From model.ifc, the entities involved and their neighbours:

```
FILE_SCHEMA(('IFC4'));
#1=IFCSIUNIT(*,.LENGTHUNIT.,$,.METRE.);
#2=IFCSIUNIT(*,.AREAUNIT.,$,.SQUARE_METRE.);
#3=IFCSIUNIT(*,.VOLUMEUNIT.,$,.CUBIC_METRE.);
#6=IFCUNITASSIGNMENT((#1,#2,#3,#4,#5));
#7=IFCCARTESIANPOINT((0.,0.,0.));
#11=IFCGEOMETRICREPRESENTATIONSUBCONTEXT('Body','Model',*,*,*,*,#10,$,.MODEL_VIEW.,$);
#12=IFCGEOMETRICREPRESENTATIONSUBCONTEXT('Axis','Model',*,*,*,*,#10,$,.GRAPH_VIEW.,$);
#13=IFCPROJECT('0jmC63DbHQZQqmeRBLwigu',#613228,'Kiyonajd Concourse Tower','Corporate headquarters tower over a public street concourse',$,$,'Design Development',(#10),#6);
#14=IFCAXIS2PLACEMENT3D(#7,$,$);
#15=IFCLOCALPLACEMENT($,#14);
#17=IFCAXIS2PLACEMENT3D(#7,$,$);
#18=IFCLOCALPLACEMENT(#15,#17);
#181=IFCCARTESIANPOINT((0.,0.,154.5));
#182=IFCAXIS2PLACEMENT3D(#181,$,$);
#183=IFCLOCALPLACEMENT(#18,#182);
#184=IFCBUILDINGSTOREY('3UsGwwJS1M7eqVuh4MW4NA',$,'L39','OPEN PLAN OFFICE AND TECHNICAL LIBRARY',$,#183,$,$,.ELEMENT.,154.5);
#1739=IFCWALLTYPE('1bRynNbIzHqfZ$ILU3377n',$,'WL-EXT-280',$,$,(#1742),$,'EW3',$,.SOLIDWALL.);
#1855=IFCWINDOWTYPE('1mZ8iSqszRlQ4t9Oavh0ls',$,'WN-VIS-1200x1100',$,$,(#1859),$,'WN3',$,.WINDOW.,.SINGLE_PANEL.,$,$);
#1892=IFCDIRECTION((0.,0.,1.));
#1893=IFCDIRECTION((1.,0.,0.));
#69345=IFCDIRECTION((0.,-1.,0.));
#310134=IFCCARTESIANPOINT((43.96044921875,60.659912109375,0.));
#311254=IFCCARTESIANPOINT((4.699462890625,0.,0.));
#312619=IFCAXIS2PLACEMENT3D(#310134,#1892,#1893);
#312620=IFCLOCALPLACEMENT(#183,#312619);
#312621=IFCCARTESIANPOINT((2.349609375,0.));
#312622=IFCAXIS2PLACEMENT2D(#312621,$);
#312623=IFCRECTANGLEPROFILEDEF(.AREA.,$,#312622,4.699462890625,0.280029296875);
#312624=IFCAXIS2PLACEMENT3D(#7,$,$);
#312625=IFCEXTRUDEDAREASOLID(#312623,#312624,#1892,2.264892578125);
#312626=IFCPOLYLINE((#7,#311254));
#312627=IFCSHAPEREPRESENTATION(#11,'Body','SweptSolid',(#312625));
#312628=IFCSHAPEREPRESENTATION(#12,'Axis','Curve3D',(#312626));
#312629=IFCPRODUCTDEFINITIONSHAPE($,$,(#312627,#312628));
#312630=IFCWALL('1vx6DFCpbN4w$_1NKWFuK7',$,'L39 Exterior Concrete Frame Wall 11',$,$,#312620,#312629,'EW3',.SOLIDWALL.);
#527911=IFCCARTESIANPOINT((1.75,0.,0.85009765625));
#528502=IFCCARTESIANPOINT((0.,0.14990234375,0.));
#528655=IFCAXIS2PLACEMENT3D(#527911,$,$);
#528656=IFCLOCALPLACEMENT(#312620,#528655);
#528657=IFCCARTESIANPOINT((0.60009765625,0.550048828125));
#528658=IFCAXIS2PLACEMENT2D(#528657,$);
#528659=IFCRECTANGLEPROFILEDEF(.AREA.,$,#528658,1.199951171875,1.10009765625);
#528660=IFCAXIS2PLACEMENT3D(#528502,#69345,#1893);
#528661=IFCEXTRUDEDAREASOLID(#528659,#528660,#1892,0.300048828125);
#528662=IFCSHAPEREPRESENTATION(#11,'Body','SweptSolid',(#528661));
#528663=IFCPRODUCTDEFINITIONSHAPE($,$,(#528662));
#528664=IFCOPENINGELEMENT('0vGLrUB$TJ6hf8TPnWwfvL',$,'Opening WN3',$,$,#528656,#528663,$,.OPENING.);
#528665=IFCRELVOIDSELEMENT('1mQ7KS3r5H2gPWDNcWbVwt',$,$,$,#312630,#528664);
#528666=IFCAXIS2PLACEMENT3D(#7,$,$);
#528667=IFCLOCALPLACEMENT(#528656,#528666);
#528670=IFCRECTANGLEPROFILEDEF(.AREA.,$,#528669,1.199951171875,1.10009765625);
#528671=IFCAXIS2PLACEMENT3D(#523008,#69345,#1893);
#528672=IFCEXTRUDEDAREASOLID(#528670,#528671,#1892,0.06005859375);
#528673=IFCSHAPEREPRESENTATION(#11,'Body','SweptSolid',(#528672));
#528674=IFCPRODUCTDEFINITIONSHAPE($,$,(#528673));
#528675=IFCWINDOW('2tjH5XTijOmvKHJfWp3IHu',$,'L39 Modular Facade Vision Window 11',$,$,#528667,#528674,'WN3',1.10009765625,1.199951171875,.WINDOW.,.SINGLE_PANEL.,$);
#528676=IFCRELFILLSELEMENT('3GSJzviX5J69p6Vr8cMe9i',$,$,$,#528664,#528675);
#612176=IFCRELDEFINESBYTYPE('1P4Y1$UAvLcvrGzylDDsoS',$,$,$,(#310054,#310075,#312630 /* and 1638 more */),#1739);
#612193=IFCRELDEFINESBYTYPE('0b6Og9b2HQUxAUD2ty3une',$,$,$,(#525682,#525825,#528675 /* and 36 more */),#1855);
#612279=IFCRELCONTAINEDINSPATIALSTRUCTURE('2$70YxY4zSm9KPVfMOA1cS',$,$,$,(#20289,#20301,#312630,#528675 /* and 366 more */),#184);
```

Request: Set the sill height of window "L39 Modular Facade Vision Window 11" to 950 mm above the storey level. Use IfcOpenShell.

```python
import numpy as np
import ifcopenshell
import ifcopenshell.api.geometry
import ifcopenshell.geom
import ifcopenshell.util.element
import ifcopenshell.util.placement
import ifcopenshell.util.shape
import ifcopenshell.util.unit

model = ifcopenshell.open("model.ifc")
unit_scale = ifcopenshell.util.unit.calculate_unit_scale(model)

window = model.by_id(528675)
opening = window.FillsVoids[0].RelatingOpeningElement
storey = ifcopenshell.util.element.get_container(window, ifc_class="IfcBuildingStorey")
level = ifcopenshell.util.placement.get_local_placement(storey.ObjectPlacement)[2, 3]

# The opening's origin need not be at the sill, so measure its lowest point.
shape = ifcopenshell.geom.create_shape(ifcopenshell.geom.settings(), opening)
bottom = ifcopenshell.util.shape.get_shape_bottom_elevation(shape, shape.geometry) / unit_scale
dz = level + 0.95 / unit_scale - bottom

shift = np.array([0.0, 0.0, dz])
# The window is placed relative to its opening, so it follows when the opening moves.
matrix = ifcopenshell.util.placement.get_local_placement(opening.ObjectPlacement)
matrix[:3, 3] += shift
ifcopenshell.api.geometry.edit_object_placement(
    model, product=opening, matrix=matrix, is_si=False, should_transform_children=True
)

print(f"moved by {dz * unit_scale:+.3f} m")

model.write("model_edited.ifc")
```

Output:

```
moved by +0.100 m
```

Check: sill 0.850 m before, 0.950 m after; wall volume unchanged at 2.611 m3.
